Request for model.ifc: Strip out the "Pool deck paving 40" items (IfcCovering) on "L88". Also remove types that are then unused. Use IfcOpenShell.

First a look at what the model holds.

```python
import ifcopenshell
import ifcopenshell.util.element

model = ifcopenshell.open("model.ifc")
print(model.schema)
storey = next(s for s in model.by_type("IfcBuildingStorey") if s.Name == "L88")
coverings = [e for e in ifcopenshell.util.element.get_decomposition(storey) if e.is_a("IfcCovering")]
seen = {}
for e in coverings:
    element_type = ifcopenshell.util.element.get_type(e)
    name = element_type.Name if element_type not in (None, e) else None
    seen[name] = seen.get(name, 0) + 1
for name, count in sorted(seen.items(), key=str):
    print(count, "x", name)
```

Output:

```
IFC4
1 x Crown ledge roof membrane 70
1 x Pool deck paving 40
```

```python
import ifcopenshell
import ifcopenshell.api.root
import ifcopenshell.util.element

model = ifcopenshell.open("model.ifc")

storey = next(s for s in model.by_type("IfcBuildingStorey") if s.Name == "L88")
coverings = [e for e in ifcopenshell.util.element.get_decomposition(storey) if e.is_a("IfcCovering")]
targets = [e for e in coverings if (t := ifcopenshell.util.element.get_type(e)) not in (None, e) and t.Name == "Pool deck paving 40"]
types = {ifcopenshell.util.element.get_type(e) for e in targets} - {None, *targets}

for e in targets:
    ifcopenshell.api.root.remove_product(model, product=e)
print(len(targets), "removed")

unused = [t for t in types if not ifcopenshell.util.element.get_types(t)]
for t in unused:
    ifcopenshell.api.root.remove_product(model, product=t)
print(len(unused), "unused types removed")

model.write("model_rev.ifc")
```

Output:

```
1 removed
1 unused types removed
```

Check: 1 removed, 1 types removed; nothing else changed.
